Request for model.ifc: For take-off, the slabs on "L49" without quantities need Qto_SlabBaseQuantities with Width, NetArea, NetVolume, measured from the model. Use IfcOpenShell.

First a look at what the model holds.

```python
import ifcopenshell
import ifcopenshell.util.element
import ifcopenshell.util.unit

model = ifcopenshell.open("model.ifc")
print(model.schema)
for unit_type in ("LENGTHUNIT", "AREAUNIT", "VOLUMEUNIT"):
    print(unit_type, ifcopenshell.util.unit.calculate_unit_scale(model, unit_type))
storey = next(s for s in model.by_type("IfcBuildingStorey") if s.Name == "L49")
slabs = [e for e in ifcopenshell.util.element.get_decomposition(storey) if e.is_a("IfcSlab")]
for e in sorted(slabs, key=lambda e: e.id()):
    print(e.id(), e.is_a(), e.Name, list(ifcopenshell.util.element.get_psets(e, qtos_only=True)), sep=" | ")
```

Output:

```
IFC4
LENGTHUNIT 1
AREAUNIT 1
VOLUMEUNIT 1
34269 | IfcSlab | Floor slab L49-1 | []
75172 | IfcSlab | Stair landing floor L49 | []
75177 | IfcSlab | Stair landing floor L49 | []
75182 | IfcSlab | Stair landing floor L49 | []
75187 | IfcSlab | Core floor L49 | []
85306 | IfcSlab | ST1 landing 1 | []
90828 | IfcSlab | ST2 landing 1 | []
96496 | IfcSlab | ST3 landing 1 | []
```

```python
import ifcopenshell
import ifcopenshell.api.pset
import ifcopenshell.geom
import ifcopenshell.util.element
import ifcopenshell.util.shape
import ifcopenshell.util.unit

model = ifcopenshell.open("model.ifc")
unit_scale = ifcopenshell.util.unit.calculate_unit_scale(model)
area_scale = ifcopenshell.util.unit.calculate_unit_scale(model, "AREAUNIT")
volume_scale = ifcopenshell.util.unit.calculate_unit_scale(model, "VOLUMEUNIT")
settings = ifcopenshell.geom.settings()

storey = next(s for s in model.by_type("IfcBuildingStorey") if s.Name == "L49")
slabs = [e for e in ifcopenshell.util.element.get_decomposition(storey) if e.is_a("IfcSlab")]

for e in sorted(slabs, key=lambda e: e.id()):
    if ifcopenshell.util.element.get_psets(e, qtos_only=True, should_inherit=False):
        continue
    # Geometry comes back in metres, in the element's own axes.
    shape = ifcopenshell.geom.create_shape(settings, e)
    values = {
        "Width": ifcopenshell.util.shape.get_z(shape.geometry) / unit_scale,
        "NetArea": ifcopenshell.util.shape.get_footprint_area(shape.geometry) / area_scale,
        "NetVolume": ifcopenshell.util.shape.get_volume(shape.geometry) / volume_scale,
    }
    qto = ifcopenshell.api.pset.add_qto(model, product=e, name="Qto_SlabBaseQuantities")
    ifcopenshell.api.pset.edit_qto(model, qto=qto, properties=values)
    print(e.id(), {k: round(v, 3) for k, v in values.items()})

model.write("model_edited.ifc")
```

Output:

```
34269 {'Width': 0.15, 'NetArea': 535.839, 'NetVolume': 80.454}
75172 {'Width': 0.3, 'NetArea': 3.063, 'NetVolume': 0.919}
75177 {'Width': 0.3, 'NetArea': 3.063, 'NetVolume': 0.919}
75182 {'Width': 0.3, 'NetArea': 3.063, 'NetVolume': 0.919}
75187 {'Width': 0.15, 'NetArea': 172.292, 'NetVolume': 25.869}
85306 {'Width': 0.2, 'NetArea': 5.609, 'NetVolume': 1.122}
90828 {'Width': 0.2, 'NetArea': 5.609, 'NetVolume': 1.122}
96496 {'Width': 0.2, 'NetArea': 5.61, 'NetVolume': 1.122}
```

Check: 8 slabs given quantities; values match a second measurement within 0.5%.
